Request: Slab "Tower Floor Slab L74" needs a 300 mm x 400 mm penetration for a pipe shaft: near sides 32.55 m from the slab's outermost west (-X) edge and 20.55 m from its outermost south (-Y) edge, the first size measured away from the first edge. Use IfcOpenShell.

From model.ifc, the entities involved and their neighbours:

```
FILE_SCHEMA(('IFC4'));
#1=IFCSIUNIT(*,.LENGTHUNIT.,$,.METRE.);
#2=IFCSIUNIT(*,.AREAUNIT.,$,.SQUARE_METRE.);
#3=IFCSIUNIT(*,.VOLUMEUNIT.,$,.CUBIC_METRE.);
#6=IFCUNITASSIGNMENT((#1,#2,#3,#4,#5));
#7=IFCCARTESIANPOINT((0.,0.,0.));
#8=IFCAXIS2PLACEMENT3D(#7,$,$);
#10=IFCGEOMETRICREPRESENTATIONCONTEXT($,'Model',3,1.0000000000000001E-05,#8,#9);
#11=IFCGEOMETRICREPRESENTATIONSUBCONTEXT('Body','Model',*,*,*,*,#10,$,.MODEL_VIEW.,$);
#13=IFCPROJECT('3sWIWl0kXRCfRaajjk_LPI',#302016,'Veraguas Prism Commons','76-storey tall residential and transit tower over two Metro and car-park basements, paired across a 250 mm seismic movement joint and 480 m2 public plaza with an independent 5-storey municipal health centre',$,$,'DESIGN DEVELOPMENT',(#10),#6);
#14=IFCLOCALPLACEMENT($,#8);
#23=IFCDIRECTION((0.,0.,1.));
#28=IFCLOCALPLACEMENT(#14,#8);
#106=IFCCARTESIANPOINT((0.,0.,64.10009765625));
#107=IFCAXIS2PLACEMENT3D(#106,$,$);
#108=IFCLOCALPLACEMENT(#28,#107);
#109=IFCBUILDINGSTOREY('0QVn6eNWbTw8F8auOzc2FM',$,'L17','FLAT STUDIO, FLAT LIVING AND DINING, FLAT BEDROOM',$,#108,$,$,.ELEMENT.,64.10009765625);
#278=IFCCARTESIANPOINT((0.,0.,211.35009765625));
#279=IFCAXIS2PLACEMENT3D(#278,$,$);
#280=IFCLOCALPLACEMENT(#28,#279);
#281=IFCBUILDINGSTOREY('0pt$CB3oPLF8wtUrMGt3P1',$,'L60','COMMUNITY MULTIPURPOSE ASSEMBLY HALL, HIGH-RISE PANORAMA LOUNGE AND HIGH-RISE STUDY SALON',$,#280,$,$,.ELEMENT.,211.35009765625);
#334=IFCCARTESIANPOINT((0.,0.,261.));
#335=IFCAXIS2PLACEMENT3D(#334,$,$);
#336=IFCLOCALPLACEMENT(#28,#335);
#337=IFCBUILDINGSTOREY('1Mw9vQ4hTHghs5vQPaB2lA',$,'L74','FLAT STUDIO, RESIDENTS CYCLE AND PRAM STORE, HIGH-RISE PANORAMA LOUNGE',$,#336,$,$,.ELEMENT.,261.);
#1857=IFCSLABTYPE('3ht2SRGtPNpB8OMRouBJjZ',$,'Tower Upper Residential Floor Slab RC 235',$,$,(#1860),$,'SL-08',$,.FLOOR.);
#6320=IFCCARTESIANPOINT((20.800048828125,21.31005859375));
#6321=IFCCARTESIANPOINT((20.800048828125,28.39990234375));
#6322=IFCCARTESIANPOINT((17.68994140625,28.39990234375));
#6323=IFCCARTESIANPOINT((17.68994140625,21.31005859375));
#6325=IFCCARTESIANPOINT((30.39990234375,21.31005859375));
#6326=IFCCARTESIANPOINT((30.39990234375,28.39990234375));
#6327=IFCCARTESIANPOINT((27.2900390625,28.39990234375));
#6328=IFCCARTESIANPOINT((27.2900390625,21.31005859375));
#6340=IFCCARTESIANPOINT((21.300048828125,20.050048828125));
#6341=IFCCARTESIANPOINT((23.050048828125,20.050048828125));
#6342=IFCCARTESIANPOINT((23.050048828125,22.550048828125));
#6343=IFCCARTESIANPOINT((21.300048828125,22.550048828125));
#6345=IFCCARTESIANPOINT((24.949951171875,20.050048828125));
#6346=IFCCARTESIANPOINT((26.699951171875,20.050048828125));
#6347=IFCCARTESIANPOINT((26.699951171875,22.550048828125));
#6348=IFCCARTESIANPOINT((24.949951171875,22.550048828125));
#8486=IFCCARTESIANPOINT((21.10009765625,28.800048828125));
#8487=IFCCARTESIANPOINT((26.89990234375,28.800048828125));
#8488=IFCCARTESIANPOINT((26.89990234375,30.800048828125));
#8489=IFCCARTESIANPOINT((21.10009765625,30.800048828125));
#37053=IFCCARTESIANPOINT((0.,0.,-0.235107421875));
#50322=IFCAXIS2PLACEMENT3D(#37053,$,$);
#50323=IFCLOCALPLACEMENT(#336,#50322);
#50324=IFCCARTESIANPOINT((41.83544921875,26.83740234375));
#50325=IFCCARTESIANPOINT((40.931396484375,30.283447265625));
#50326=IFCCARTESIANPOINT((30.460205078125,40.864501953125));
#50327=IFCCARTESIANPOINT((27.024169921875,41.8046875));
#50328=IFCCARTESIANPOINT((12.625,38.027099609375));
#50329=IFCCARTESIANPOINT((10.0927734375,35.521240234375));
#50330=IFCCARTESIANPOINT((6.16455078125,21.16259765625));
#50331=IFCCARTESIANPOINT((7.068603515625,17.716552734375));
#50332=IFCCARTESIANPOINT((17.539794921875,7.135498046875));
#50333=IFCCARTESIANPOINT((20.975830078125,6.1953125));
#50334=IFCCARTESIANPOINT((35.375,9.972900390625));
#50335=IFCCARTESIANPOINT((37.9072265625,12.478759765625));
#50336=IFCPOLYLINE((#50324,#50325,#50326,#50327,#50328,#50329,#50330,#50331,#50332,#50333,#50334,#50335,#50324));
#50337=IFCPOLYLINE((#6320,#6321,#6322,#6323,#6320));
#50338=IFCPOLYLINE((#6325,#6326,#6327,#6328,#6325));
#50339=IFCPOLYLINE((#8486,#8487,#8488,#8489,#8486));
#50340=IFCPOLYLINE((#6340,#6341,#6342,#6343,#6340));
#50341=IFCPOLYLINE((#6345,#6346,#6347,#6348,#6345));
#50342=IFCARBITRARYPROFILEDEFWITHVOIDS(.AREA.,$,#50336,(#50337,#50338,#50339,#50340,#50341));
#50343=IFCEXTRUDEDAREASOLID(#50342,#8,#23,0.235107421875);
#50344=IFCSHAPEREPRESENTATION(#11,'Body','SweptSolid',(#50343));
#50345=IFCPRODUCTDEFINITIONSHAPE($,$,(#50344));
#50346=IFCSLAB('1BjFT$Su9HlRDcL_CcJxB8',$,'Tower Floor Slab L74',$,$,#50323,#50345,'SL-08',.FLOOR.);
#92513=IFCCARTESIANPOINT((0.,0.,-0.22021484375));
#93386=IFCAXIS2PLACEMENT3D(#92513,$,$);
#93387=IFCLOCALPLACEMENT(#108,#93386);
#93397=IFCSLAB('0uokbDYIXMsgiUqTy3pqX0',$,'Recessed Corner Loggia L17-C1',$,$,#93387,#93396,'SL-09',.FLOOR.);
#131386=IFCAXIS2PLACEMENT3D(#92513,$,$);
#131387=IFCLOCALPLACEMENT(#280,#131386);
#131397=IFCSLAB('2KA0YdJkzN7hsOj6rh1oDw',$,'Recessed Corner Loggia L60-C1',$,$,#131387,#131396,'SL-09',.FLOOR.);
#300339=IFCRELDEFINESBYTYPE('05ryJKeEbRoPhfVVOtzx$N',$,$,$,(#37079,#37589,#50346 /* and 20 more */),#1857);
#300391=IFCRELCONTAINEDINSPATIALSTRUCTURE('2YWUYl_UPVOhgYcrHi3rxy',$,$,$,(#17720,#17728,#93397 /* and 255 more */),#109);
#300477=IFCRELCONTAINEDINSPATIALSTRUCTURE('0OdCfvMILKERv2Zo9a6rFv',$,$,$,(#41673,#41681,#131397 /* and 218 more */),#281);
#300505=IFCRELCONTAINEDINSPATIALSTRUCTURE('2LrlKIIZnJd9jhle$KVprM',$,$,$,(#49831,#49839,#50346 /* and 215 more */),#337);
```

```python
import numpy as np
import ifcopenshell
import ifcopenshell.api.feature
import ifcopenshell.api.geometry
import ifcopenshell.api.root
import ifcopenshell.geom
import ifcopenshell.util.placement
import ifcopenshell.util.representation
import ifcopenshell.util.shape
import ifcopenshell.util.unit

model = ifcopenshell.open("model.ifc")
unit_scale = ifcopenshell.util.unit.calculate_unit_scale(model)
settings = ifcopenshell.geom.settings()


def volume(element):
    """Net volume in cubic metres, openings subtracted."""
    shape = ifcopenshell.geom.create_shape(settings, element)
    return ifcopenshell.util.shape.get_volume(shape.geometry)


slab = model.by_guid("1BjFT$Su9HlRDcL_CcJxB8")
before = volume(slab)

# Extent in the slab's own axes, in metres. The edges named are its -X and -Y sides.
slab_shape = ifcopenshell.geom.create_shape(settings, slab)
vertices = ifcopenshell.util.shape.get_vertices(slab_shape.geometry)
x_min, y_min, bottom = vertices.min(axis=0)
top = vertices[:, 2].max()

opening = ifcopenshell.api.root.create_entity(model, ifc_class="IfcOpeningElement", name="Pipe shaft opening", predefined_type="OPENING")
context = ifcopenshell.util.representation.get_context(model, "Model", "Body", "MODEL_VIEW")
width, depth = 0.3, 0.4
outline = [(0.0, 0.0), (width, 0.0), (width, depth), (0.0, depth), (0.0, 0.0)]
# Overshoot both faces by 50 mm so the cut is clean.
shape = ifcopenshell.api.geometry.add_slab_representation(
    model, context=context, depth=top - bottom + 0.1, polyline=outline
)
ifcopenshell.api.geometry.assign_representation(model, product=opening, representation=shape)

matrix = ifcopenshell.util.placement.get_local_placement(slab.ObjectPlacement)
matrix[:, 3] = matrix @ np.append(np.array([x_min + 32.55, y_min + 20.55, bottom - 0.05]) / unit_scale, 1.0)
ifcopenshell.api.geometry.edit_object_placement(model, product=opening, matrix=matrix, is_si=False)
ifcopenshell.api.feature.add_feature(model, feature=opening, element=slab)

after = volume(slab)

print(f"slab volume {before:.3f} -> {after:.3f} m3")

model.write("model_v2.ifc")
```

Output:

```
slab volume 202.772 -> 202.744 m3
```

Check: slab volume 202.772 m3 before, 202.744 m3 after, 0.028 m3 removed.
